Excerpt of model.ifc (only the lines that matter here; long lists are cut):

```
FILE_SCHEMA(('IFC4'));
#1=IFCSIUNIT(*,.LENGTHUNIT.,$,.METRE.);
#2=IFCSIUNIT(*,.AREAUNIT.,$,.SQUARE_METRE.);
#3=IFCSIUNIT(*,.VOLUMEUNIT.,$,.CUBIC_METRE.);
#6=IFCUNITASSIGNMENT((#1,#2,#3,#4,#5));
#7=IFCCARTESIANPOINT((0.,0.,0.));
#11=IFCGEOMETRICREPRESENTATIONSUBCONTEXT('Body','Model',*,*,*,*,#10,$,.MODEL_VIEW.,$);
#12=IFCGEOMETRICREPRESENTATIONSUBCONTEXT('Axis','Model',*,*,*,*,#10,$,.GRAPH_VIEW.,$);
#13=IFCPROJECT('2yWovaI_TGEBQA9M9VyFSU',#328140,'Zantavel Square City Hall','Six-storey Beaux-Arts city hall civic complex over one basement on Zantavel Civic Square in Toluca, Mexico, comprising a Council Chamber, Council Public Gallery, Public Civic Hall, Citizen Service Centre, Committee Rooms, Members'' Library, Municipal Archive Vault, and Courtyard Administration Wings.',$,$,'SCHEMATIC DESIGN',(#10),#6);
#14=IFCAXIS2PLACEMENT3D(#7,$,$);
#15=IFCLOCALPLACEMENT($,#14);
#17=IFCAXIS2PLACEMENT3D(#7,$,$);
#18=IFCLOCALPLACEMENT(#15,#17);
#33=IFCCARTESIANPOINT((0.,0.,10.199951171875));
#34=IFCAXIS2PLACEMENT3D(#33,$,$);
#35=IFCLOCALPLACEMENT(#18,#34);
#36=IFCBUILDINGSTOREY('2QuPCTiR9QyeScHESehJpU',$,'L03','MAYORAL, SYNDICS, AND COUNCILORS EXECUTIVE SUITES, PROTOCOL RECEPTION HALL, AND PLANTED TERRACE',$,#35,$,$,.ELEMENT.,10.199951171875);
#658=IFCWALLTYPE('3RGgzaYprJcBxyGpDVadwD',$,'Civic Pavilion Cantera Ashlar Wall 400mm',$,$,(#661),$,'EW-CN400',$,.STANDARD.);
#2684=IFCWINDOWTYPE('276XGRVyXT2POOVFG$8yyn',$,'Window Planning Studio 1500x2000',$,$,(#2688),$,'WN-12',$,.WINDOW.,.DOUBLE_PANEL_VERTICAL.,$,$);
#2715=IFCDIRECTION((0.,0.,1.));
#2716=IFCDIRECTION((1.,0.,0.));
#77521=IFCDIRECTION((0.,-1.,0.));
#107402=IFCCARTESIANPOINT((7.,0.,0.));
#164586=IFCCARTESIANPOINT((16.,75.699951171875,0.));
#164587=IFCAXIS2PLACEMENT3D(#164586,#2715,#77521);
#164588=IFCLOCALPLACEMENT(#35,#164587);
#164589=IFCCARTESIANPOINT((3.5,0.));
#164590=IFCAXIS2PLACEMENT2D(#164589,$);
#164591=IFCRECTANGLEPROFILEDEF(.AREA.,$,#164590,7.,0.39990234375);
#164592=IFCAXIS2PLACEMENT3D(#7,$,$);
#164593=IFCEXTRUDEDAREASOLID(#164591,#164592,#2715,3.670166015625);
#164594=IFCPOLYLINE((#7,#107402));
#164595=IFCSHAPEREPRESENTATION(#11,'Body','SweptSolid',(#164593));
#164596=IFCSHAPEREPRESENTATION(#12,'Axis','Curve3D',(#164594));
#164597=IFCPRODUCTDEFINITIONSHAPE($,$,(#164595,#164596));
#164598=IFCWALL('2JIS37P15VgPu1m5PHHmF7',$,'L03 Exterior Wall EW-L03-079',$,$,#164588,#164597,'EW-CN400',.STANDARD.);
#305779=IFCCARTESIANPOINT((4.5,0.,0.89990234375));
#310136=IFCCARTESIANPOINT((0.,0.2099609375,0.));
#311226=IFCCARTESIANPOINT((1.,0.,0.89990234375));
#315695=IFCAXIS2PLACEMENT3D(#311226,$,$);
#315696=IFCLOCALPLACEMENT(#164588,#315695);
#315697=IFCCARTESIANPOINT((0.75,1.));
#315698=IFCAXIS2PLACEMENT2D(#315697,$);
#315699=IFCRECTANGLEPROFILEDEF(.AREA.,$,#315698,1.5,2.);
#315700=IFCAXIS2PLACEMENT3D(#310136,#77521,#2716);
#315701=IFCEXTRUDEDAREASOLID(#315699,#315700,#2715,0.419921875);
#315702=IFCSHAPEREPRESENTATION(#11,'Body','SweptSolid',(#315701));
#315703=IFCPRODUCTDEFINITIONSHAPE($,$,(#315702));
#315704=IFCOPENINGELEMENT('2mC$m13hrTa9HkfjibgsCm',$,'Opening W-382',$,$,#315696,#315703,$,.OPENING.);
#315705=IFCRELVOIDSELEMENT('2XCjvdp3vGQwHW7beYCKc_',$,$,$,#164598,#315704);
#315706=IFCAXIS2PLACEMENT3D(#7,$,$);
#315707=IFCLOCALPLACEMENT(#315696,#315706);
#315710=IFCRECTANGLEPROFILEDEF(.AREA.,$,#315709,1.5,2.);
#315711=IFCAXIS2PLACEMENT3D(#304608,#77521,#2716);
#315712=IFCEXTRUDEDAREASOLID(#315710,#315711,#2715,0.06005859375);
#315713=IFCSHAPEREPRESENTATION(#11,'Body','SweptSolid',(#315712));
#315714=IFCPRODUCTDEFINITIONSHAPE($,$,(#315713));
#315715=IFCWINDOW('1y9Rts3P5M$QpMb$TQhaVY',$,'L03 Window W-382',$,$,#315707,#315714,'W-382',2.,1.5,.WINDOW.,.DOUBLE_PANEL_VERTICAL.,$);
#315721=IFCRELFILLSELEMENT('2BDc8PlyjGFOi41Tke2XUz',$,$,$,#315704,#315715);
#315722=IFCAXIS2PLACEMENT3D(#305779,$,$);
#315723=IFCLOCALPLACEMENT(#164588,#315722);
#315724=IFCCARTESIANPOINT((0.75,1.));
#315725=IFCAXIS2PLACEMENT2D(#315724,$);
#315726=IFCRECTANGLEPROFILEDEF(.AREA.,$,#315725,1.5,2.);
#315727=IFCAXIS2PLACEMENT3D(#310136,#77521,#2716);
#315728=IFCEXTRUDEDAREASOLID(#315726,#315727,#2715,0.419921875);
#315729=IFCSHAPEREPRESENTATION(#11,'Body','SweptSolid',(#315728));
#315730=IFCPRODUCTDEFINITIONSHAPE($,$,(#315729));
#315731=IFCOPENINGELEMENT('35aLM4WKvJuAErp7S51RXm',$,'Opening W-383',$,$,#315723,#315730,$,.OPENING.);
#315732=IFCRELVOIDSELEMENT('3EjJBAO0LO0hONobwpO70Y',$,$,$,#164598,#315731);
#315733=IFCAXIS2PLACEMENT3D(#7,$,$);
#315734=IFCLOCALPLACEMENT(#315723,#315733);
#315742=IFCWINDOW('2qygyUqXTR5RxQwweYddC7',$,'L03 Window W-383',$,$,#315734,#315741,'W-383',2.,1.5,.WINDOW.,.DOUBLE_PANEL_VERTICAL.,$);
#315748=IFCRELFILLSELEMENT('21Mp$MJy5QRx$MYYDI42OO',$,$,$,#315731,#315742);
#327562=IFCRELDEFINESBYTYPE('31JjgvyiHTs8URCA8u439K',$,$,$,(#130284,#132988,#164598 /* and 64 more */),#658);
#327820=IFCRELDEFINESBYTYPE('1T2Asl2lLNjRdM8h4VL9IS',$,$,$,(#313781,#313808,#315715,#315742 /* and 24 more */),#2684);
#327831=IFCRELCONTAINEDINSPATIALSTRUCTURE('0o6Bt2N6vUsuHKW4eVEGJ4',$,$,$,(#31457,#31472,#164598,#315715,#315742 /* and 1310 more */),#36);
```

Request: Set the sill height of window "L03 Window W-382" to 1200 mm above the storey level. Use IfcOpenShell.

```python
import numpy as np
import ifcopenshell
import ifcopenshell.api.geometry
import ifcopenshell.geom
import ifcopenshell.util.element
import ifcopenshell.util.placement
import ifcopenshell.util.shape
import ifcopenshell.util.unit

model = ifcopenshell.open("model.ifc")
unit_scale = ifcopenshell.util.unit.calculate_unit_scale(model)

window = model.by_guid("1y9Rts3P5M$QpMb$TQhaVY")
opening = window.FillsVoids[0].RelatingOpeningElement
storey = ifcopenshell.util.element.get_container(window, ifc_class="IfcBuildingStorey")
level = ifcopenshell.util.placement.get_local_placement(storey.ObjectPlacement)[2, 3]

# The opening's origin need not be at the sill, so measure its lowest point.
shape = ifcopenshell.geom.create_shape(ifcopenshell.geom.settings(), opening)
bottom = ifcopenshell.util.shape.get_shape_bottom_elevation(shape, shape.geometry) / unit_scale
dz = level + 1.2 - bottom

shift = np.array([0.0, 0.0, dz])
# The window is placed relative to its opening, so it follows when the opening moves.
matrix = ifcopenshell.util.placement.get_local_placement(opening.ObjectPlacement)
matrix[:3, 3] += shift
ifcopenshell.api.geometry.edit_object_placement(
    model, product=opening, matrix=matrix, is_si=False, should_transform_children=True
)

print(f"moved by {dz * unit_scale:+.3f} m")

model.write("model-out.ifc")
```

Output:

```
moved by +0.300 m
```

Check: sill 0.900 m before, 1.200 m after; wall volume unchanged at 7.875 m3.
